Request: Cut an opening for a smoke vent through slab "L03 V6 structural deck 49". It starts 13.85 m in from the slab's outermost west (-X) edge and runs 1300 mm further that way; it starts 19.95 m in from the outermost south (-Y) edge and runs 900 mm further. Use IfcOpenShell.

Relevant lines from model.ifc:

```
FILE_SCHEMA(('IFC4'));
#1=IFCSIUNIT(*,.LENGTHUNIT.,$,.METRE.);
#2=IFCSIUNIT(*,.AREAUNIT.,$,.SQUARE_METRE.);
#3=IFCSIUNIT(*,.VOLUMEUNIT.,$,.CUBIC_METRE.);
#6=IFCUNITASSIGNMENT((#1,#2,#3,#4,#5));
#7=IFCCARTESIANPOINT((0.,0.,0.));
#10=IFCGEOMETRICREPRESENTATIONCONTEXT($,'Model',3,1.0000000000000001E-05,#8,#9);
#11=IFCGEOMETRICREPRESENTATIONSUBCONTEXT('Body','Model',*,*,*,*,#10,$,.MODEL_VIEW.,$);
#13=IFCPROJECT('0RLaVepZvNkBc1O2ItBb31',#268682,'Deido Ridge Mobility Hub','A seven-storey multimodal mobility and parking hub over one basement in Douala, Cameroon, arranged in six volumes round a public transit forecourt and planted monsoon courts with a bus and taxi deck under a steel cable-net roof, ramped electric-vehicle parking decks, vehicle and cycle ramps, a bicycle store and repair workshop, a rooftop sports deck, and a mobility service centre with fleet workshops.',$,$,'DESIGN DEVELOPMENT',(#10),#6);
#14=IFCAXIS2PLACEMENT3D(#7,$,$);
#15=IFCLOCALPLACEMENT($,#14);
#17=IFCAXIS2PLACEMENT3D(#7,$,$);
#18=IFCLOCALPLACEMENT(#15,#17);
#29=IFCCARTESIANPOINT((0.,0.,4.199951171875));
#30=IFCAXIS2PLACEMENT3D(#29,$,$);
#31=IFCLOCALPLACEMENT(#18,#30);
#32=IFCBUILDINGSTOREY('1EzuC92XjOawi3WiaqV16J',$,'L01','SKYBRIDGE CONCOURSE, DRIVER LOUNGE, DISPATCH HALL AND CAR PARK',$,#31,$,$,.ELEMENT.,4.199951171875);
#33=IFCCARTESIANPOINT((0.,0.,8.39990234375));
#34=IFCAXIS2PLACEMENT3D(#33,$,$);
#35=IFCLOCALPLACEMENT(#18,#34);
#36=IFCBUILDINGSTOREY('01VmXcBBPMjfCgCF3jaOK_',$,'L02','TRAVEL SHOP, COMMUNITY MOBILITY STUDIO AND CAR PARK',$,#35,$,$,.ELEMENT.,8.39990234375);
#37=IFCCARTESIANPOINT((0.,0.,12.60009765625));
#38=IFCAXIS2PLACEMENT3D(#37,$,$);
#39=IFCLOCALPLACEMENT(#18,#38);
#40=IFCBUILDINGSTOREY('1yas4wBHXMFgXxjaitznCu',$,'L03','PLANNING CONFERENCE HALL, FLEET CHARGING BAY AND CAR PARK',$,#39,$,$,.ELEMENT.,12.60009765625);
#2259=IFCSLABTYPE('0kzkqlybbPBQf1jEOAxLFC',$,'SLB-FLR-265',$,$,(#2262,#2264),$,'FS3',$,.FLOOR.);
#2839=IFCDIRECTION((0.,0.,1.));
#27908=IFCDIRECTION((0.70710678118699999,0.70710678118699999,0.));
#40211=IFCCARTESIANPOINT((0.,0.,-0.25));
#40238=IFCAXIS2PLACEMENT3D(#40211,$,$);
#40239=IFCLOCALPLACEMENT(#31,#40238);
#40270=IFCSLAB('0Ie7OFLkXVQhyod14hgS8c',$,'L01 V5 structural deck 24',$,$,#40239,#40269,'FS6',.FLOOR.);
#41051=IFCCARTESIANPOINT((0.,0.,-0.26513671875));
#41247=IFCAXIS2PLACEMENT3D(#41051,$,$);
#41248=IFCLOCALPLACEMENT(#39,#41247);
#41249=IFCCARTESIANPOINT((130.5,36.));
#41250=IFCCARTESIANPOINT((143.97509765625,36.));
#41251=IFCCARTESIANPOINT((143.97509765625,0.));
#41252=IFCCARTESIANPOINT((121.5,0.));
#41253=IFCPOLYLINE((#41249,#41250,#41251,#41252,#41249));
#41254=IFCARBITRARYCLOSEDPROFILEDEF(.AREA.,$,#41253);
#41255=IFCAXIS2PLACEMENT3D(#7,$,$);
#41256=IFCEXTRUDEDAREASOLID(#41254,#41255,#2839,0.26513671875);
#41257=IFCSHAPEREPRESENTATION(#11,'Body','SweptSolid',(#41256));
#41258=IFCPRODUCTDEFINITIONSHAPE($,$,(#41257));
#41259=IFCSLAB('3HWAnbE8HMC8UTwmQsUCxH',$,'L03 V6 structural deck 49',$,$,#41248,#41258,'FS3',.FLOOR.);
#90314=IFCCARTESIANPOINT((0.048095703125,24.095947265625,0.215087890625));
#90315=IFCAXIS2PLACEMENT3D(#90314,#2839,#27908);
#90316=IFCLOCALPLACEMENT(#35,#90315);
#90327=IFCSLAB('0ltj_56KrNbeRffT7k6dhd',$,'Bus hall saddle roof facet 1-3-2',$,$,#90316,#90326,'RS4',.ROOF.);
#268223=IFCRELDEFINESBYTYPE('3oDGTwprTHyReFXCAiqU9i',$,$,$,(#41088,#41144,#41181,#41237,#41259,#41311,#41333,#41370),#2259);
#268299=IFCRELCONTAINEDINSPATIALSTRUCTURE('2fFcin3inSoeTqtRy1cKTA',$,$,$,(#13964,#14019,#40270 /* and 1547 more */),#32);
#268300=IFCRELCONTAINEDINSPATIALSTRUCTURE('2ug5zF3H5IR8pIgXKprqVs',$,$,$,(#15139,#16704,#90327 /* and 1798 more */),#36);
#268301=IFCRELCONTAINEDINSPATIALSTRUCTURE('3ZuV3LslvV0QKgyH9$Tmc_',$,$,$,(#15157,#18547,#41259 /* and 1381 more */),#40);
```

```python
import numpy as np
import ifcopenshell
import ifcopenshell.api.feature
import ifcopenshell.api.geometry
import ifcopenshell.api.root
import ifcopenshell.geom
import ifcopenshell.util.placement
import ifcopenshell.util.representation
import ifcopenshell.util.shape
import ifcopenshell.util.unit

model = ifcopenshell.open("model.ifc")
unit_scale = ifcopenshell.util.unit.calculate_unit_scale(model)
settings = ifcopenshell.geom.settings()


def volume(element):
    """Net volume in cubic metres, openings subtracted."""
    shape = ifcopenshell.geom.create_shape(settings, element)
    return ifcopenshell.util.shape.get_volume(shape.geometry)


slab = model.by_id(41259)
before = volume(slab)

# Extent in the slab's own axes, in metres. The edges named are its -X and -Y sides.
slab_shape = ifcopenshell.geom.create_shape(settings, slab)
vertices = ifcopenshell.util.shape.get_vertices(slab_shape.geometry)
x_min, y_min, bottom = vertices.min(axis=0)
top = vertices[:, 2].max()

opening = ifcopenshell.api.root.create_entity(model, ifc_class="IfcOpeningElement", name="Smoke vent opening", predefined_type="OPENING")
context = ifcopenshell.util.representation.get_context(model, "Model", "Body", "MODEL_VIEW")
width, depth = 1.3, 0.9
outline = [(0.0, 0.0), (width, 0.0), (width, depth), (0.0, depth), (0.0, 0.0)]
# Overshoot both faces by 50 mm so the cut is clean.
shape = ifcopenshell.api.geometry.add_slab_representation(
    model, context=context, depth=top - bottom + 0.1, polyline=outline
)
ifcopenshell.api.geometry.assign_representation(model, product=opening, representation=shape)

matrix = ifcopenshell.util.placement.get_local_placement(slab.ObjectPlacement)
matrix[:, 3] = matrix @ np.append(np.array([x_min + 13.85, y_min + 19.95, bottom - 0.05]) / unit_scale, 1.0)
ifcopenshell.api.geometry.edit_object_placement(model, product=opening, matrix=matrix, is_si=False)
ifcopenshell.api.feature.add_feature(model, feature=opening, element=slab)

after = volume(slab)

print(f"slab volume {before:.3f} -> {after:.3f} m3")

model.write("model_updated.ifc")
```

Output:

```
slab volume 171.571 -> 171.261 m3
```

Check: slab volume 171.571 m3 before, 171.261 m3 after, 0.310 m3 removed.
